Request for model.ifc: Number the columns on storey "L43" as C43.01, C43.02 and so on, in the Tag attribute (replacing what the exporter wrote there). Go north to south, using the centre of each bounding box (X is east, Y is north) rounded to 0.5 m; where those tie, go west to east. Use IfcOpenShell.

First a look at what the model holds.

```python
import ifcopenshell
import ifcopenshell.util.element
import ifcopenshell.util.placement

model = ifcopenshell.open("model.ifc")
print(model.schema)
storey = next(s for s in model.by_type("IfcBuildingStorey") if s.Name == "L43")
columns = [e for e in ifcopenshell.util.element.get_decomposition(storey) if e.is_a("IfcColumn")]
for e in sorted(columns, key=lambda e: e.id()):
    origin = ifcopenshell.util.placement.get_local_placement(e.ObjectPlacement)[:3, 3]
    print(e.id(), e.Tag, e.Name, origin.round(2) + 0.0, sep=" | ")
```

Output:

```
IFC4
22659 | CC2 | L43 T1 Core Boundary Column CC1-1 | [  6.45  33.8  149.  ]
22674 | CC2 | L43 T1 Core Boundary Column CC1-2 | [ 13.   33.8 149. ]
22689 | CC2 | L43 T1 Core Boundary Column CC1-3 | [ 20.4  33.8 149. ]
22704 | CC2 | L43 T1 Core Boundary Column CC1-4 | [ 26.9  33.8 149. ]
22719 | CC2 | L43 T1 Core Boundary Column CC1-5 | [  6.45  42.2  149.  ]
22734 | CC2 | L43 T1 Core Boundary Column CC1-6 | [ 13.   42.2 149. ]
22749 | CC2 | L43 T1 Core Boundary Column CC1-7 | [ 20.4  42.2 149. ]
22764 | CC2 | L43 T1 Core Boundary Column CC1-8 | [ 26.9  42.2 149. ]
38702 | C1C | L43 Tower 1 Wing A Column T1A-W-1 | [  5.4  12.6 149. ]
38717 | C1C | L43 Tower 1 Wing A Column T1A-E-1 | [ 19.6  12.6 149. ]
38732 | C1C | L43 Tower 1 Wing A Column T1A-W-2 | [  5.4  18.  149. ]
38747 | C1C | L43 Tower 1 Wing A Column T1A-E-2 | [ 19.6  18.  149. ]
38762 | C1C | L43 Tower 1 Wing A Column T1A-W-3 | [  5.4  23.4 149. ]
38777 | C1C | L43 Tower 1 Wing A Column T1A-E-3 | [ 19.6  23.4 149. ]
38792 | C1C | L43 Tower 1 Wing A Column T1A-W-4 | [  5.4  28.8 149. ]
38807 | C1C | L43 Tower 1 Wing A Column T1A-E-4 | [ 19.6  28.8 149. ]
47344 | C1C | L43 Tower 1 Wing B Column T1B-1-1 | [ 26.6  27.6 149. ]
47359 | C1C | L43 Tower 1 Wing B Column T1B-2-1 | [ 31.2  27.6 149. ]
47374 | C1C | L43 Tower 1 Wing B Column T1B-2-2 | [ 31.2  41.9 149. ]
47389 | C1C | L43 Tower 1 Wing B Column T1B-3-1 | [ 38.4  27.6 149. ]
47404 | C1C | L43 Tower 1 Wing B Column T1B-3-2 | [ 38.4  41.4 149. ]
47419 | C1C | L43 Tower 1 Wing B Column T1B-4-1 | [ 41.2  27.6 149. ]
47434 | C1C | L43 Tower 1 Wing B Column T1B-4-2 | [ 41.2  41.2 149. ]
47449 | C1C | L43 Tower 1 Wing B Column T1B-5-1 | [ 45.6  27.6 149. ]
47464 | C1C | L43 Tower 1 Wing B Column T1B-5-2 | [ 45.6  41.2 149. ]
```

```python
import ifcopenshell
import ifcopenshell.geom
import ifcopenshell.util.element
import ifcopenshell.util.shape

model = ifcopenshell.open("model.ifc")
settings = ifcopenshell.geom.settings()
settings.set("use-world-coords", True)


def centre(element):
    shape = ifcopenshell.geom.create_shape(settings, element)
    return ifcopenshell.util.shape.get_bbox_centroid(shape.geometry)


storey = next(s for s in model.by_type("IfcBuildingStorey") if s.Name == "L43")
columns = [e for e in ifcopenshell.util.element.get_decomposition(storey) if e.is_a("IfcColumn")]

# Insertion points can sit at a corner or the storey origin, so sort by the geometry (in metres).
centres = {e: centre(e) for e in columns}
columns.sort(key=lambda e: (-round(centres[e][1] / 0.5), centres[e][0]))

for i, e in enumerate(columns, start=1):
    number = f"C43.{i:02d}"
    e.Tag = number
    print(e.id(), number)

model.write("model_v2.ifc")
```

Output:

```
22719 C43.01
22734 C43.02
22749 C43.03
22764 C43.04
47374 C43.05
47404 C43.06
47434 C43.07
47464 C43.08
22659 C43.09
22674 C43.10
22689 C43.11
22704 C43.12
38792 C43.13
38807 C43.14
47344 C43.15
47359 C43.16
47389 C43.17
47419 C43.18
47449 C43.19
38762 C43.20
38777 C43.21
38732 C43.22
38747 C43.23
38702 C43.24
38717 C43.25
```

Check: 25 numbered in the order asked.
